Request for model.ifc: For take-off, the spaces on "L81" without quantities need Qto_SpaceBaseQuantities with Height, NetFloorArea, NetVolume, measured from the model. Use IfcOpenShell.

First a look at what the model holds.

```python
import ifcopenshell
import ifcopenshell.util.element
import ifcopenshell.util.unit

model = ifcopenshell.open("model.ifc")
print(model.schema)
for unit_type in ("LENGTHUNIT", "AREAUNIT", "VOLUMEUNIT"):
    print(unit_type, ifcopenshell.util.unit.calculate_unit_scale(model, unit_type))
storey = next(s for s in model.by_type("IfcBuildingStorey") if s.Name == "L81")
spaces = [e for e in ifcopenshell.util.element.get_decomposition(storey) if e.is_a("IfcSpace")]
for e in sorted(spaces, key=lambda e: e.id()):
    print(e.id(), e.is_a(), e.Name, list(ifcopenshell.util.element.get_psets(e, qtos_only=True)), sep=" | ")
```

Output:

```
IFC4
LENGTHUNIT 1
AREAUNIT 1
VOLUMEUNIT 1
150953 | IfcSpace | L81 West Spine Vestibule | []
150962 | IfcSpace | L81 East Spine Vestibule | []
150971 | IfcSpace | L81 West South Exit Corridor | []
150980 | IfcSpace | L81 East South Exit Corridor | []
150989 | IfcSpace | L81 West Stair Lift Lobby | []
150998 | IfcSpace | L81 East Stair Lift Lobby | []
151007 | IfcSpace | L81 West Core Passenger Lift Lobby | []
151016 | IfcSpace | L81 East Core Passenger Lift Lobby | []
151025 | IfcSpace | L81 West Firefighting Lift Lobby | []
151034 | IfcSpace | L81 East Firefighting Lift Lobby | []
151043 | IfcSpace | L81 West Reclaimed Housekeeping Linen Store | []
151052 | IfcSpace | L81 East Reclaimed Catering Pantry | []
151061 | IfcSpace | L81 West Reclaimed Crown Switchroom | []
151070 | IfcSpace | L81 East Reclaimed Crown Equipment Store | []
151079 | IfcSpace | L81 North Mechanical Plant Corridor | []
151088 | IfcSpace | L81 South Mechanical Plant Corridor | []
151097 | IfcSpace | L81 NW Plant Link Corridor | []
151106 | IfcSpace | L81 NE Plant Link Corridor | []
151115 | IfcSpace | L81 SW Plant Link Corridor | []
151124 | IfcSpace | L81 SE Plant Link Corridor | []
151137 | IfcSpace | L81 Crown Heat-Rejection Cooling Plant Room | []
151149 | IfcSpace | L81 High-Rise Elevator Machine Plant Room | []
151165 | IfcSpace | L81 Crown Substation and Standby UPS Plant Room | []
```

```python
import ifcopenshell
import ifcopenshell.api.pset
import ifcopenshell.geom
import ifcopenshell.util.element
import ifcopenshell.util.shape
import ifcopenshell.util.unit

model = ifcopenshell.open("model.ifc")
unit_scale = ifcopenshell.util.unit.calculate_unit_scale(model)
area_scale = ifcopenshell.util.unit.calculate_unit_scale(model, "AREAUNIT")
volume_scale = ifcopenshell.util.unit.calculate_unit_scale(model, "VOLUMEUNIT")
settings = ifcopenshell.geom.settings()

storey = next(s for s in model.by_type("IfcBuildingStorey") if s.Name == "L81")
spaces = [e for e in ifcopenshell.util.element.get_decomposition(storey) if e.is_a("IfcSpace")]

for e in sorted(spaces, key=lambda e: e.id()):
    if ifcopenshell.util.element.get_psets(e, qtos_only=True, should_inherit=False):
        continue
    # Geometry comes back in metres, in the element's own axes.
    shape = ifcopenshell.geom.create_shape(settings, e)
    values = {
        "Height": ifcopenshell.util.shape.get_z(shape.geometry) / unit_scale,
        "NetFloorArea": ifcopenshell.util.shape.get_footprint_area(shape.geometry) / area_scale,
        "NetVolume": ifcopenshell.util.shape.get_volume(shape.geometry) / volume_scale,
    }
    qto = ifcopenshell.api.pset.add_qto(model, product=e, name="Qto_SpaceBaseQuantities")
    ifcopenshell.api.pset.edit_qto(model, qto=qto, properties=values)
    print(e.id(), {k: round(v, 3) for k, v in values.items()})

model.write("model_updated.ifc")
```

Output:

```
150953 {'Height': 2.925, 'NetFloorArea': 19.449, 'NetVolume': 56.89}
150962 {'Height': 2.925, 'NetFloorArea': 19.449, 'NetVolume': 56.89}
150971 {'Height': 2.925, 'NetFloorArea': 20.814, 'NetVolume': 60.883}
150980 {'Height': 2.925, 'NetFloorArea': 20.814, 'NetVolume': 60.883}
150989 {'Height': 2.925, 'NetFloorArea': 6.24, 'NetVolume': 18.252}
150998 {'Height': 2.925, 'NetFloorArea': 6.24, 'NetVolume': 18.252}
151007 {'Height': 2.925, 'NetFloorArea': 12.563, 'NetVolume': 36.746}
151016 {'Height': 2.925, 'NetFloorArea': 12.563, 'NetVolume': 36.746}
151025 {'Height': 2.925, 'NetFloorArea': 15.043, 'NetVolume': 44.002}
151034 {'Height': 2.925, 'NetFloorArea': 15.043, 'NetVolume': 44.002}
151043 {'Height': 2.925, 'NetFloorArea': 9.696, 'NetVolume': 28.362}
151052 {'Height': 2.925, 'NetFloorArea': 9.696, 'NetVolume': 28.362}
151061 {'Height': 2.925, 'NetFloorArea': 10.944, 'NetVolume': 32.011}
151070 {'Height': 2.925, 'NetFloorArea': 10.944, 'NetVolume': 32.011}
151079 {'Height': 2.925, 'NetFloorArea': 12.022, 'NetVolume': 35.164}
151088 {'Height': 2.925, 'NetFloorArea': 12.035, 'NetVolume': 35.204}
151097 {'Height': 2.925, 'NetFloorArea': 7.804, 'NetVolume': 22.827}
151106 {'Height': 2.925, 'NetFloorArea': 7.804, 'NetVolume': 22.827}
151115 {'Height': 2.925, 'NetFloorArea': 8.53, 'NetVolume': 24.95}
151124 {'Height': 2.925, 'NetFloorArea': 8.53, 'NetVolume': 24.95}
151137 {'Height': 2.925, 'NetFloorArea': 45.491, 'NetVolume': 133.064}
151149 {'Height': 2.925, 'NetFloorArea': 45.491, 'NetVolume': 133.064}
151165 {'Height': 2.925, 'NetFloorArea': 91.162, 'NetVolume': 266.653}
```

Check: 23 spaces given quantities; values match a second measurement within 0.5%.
